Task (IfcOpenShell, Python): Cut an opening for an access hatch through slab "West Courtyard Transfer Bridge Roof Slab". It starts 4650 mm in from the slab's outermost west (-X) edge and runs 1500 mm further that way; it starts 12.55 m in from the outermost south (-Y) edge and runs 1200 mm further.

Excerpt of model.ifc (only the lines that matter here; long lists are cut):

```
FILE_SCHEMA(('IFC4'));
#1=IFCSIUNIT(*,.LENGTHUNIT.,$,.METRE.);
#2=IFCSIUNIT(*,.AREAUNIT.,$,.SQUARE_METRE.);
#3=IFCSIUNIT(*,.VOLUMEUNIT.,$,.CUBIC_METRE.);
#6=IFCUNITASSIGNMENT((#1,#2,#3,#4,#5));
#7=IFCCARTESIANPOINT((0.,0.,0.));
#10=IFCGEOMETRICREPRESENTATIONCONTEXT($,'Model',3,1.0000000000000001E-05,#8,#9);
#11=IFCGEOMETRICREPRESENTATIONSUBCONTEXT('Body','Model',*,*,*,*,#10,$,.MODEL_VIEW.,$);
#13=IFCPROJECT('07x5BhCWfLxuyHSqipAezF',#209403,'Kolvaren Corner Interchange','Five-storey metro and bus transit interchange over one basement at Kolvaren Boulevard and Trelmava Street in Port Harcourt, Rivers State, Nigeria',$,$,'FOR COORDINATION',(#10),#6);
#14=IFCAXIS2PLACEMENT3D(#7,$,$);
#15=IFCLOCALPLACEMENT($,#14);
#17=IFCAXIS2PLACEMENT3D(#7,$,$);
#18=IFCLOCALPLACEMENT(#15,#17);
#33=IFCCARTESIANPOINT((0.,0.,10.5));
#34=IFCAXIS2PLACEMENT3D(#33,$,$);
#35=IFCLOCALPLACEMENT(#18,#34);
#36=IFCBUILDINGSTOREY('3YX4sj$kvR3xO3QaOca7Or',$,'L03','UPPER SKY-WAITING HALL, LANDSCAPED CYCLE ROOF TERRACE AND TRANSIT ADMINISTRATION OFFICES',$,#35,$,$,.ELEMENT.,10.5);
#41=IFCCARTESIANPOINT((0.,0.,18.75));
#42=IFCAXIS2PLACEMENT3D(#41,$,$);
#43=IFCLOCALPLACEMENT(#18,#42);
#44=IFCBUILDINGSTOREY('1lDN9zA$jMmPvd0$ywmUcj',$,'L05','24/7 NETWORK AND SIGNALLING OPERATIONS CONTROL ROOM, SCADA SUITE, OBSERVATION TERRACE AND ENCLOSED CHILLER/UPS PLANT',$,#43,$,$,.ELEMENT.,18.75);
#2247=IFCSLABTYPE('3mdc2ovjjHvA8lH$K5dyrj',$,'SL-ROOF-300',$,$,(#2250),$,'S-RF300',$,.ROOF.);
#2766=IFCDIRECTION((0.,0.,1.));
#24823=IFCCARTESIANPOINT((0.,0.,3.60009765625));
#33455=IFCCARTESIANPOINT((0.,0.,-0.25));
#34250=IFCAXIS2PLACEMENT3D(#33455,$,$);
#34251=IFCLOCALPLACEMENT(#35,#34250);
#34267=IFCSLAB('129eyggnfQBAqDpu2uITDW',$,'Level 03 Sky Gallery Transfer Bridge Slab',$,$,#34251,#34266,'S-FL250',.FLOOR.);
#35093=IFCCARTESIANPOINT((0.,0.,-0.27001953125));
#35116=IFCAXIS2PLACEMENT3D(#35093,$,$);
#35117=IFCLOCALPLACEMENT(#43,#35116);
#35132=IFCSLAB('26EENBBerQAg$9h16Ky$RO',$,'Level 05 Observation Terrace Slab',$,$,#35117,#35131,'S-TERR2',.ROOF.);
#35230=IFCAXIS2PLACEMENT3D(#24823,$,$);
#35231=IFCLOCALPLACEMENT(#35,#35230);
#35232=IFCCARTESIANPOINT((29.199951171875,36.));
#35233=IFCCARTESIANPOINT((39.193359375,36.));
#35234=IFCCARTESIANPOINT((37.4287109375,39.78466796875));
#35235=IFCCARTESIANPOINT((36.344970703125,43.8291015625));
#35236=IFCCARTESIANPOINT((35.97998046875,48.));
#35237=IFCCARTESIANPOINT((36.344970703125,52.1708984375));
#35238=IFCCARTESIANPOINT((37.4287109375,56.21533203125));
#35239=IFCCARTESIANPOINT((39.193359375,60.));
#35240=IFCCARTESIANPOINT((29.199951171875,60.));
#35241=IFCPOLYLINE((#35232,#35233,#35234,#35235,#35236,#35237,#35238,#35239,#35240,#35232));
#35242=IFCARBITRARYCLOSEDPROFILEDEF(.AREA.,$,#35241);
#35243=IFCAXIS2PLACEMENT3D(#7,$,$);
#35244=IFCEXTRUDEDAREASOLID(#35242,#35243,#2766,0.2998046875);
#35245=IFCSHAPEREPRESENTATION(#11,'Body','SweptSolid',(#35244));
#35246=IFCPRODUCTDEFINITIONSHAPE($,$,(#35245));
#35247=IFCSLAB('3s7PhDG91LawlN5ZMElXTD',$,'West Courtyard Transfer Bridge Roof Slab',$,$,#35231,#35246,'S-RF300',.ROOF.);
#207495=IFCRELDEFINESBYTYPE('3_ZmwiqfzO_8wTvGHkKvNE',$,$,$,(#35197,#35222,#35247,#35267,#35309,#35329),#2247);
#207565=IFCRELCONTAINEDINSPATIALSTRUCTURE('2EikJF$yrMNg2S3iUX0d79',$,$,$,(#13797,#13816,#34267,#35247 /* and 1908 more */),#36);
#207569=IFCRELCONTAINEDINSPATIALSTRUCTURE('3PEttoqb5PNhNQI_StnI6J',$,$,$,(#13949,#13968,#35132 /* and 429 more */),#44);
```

```python
import numpy as np
import ifcopenshell
import ifcopenshell.api.feature
import ifcopenshell.api.geometry
import ifcopenshell.api.root
import ifcopenshell.geom
import ifcopenshell.util.placement
import ifcopenshell.util.representation
import ifcopenshell.util.shape
import ifcopenshell.util.unit

model = ifcopenshell.open("model.ifc")
unit_scale = ifcopenshell.util.unit.calculate_unit_scale(model)
settings = ifcopenshell.geom.settings()


def volume(element):
    """Net volume in cubic metres, openings subtracted."""
    shape = ifcopenshell.geom.create_shape(settings, element)
    return ifcopenshell.util.shape.get_volume(shape.geometry)


slab = model.by_guid("3s7PhDG91LawlN5ZMElXTD")
before = volume(slab)

# Extent in the slab's own axes, in metres. The edges named are its -X and -Y sides.
slab_shape = ifcopenshell.geom.create_shape(settings, slab)
vertices = ifcopenshell.util.shape.get_vertices(slab_shape.geometry)
x_min, y_min, bottom = vertices.min(axis=0)
top = vertices[:, 2].max()

opening = ifcopenshell.api.root.create_entity(model, ifc_class="IfcOpeningElement", name="Access hatch opening", predefined_type="OPENING")
context = ifcopenshell.util.representation.get_context(model, "Model", "Body", "MODEL_VIEW")
width, depth = 1.5, 1.2
outline = [(0.0, 0.0), (width, 0.0), (width, depth), (0.0, depth), (0.0, 0.0)]
# Overshoot both faces by 50 mm so the cut is clean.
shape = ifcopenshell.api.geometry.add_slab_representation(
    model, context=context, depth=top - bottom + 0.1, polyline=outline
)
ifcopenshell.api.geometry.assign_representation(model, product=opening, representation=shape)

matrix = ifcopenshell.util.placement.get_local_placement(slab.ObjectPlacement)
matrix[:, 3] = matrix @ np.append(np.array([x_min + 4.65, y_min + 12.55, bottom - 0.05]) / unit_scale, 1.0)
ifcopenshell.api.geometry.edit_object_placement(model, product=opening, matrix=matrix, is_si=False)
ifcopenshell.api.feature.add_feature(model, feature=opening, element=slab)

after = volume(slab)

print(f"slab volume {before:.3f} -> {after:.3f} m3")

model.write("model_edited.ifc")
```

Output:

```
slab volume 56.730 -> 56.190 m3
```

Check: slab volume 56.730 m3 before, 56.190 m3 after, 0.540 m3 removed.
